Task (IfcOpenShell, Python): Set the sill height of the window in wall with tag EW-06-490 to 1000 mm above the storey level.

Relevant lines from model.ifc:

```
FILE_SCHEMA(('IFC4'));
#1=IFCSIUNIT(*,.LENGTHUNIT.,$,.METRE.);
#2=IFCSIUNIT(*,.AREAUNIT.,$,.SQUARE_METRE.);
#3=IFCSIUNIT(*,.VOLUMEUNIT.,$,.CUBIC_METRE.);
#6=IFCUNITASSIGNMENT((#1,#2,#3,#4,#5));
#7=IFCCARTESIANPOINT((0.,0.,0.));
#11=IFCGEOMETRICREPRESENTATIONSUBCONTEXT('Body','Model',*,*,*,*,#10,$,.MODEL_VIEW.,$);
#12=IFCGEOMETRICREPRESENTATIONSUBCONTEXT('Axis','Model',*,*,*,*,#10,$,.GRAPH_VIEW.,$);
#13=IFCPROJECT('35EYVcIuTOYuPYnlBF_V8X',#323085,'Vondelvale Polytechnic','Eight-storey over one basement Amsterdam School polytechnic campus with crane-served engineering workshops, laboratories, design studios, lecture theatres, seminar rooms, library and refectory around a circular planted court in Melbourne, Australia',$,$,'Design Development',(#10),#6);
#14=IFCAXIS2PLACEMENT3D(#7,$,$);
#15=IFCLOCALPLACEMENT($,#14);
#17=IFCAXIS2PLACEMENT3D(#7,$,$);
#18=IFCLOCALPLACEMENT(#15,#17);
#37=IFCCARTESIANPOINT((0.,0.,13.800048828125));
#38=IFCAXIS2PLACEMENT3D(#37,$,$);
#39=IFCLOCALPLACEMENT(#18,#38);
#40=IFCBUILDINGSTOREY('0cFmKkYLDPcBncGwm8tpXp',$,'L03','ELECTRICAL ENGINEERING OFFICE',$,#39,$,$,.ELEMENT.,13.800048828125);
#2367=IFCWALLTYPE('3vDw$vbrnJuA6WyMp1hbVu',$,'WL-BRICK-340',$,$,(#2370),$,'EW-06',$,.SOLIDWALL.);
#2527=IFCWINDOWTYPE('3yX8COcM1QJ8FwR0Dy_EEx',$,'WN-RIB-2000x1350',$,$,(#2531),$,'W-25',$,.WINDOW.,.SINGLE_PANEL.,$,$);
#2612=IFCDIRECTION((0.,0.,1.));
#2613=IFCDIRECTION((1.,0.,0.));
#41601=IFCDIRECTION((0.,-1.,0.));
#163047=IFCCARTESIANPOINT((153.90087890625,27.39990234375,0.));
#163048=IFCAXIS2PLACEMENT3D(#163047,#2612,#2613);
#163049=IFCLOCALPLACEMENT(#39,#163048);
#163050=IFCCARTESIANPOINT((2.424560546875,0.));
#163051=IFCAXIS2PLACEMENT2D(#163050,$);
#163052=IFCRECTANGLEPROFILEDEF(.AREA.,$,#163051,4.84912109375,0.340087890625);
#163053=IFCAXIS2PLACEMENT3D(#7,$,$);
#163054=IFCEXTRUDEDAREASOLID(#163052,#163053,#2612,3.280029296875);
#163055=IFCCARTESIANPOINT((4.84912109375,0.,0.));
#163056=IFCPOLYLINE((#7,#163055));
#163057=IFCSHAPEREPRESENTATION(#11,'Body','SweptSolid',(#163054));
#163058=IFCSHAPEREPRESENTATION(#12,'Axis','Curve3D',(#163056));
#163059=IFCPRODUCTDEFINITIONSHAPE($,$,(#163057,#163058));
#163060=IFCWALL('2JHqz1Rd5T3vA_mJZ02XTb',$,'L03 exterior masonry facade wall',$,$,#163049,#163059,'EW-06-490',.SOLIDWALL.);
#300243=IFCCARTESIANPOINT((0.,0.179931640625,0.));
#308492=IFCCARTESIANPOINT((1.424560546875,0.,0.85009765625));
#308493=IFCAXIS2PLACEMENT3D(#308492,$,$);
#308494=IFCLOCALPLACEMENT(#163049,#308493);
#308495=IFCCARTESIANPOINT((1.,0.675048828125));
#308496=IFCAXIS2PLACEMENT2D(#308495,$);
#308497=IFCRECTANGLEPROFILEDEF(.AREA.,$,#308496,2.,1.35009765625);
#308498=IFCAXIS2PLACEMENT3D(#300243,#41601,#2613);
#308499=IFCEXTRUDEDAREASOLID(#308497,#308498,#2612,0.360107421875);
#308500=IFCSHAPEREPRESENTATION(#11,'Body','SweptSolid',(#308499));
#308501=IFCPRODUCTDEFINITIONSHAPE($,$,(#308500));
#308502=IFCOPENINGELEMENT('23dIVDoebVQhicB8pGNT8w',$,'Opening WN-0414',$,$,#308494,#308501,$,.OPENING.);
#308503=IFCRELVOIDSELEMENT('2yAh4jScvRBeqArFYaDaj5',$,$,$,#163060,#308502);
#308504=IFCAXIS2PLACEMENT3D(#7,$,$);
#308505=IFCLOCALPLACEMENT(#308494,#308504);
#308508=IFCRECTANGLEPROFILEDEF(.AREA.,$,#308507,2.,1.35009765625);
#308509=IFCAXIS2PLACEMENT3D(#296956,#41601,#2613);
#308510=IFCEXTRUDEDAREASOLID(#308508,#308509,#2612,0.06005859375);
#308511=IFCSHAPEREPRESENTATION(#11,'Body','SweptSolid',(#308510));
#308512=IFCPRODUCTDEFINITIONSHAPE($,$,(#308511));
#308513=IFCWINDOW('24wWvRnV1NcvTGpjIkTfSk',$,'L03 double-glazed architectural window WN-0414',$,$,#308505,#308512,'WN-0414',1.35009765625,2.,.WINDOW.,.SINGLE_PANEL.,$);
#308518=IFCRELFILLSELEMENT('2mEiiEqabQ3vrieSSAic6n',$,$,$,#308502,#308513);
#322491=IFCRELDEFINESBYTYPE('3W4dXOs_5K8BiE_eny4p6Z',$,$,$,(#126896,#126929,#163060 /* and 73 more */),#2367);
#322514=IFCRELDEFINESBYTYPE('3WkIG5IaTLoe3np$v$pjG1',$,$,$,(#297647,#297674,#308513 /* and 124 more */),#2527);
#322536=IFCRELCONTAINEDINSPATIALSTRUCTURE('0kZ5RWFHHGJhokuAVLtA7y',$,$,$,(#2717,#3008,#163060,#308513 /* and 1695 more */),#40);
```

```python
import numpy as np
import ifcopenshell
import ifcopenshell.api.geometry
import ifcopenshell.geom
import ifcopenshell.util.element
import ifcopenshell.util.placement
import ifcopenshell.util.shape
import ifcopenshell.util.unit

model = ifcopenshell.open("model.ifc")
unit_scale = ifcopenshell.util.unit.calculate_unit_scale(model)

window = model.by_id(308513)
opening = window.FillsVoids[0].RelatingOpeningElement
storey = ifcopenshell.util.element.get_container(window, ifc_class="IfcBuildingStorey")
level = ifcopenshell.util.placement.get_local_placement(storey.ObjectPlacement)[2, 3]

# The opening's origin need not be at the sill, so measure its lowest point.
shape = ifcopenshell.geom.create_shape(ifcopenshell.geom.settings(), opening)
bottom = ifcopenshell.util.shape.get_shape_bottom_elevation(shape, shape.geometry) / unit_scale
dz = level + 1 / unit_scale - bottom

shift = np.array([0.0, 0.0, dz])
# The window is placed relative to its opening, so it follows when the opening moves.
matrix = ifcopenshell.util.placement.get_local_placement(opening.ObjectPlacement)
matrix[:3, 3] += shift
ifcopenshell.api.geometry.edit_object_placement(
    model, product=opening, matrix=matrix, is_si=False, should_transform_children=True
)

print(f"moved by {dz * unit_scale:+.3f} m")

model.write("model_v2.ifc")
```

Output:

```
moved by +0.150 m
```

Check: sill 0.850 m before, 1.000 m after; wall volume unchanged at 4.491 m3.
